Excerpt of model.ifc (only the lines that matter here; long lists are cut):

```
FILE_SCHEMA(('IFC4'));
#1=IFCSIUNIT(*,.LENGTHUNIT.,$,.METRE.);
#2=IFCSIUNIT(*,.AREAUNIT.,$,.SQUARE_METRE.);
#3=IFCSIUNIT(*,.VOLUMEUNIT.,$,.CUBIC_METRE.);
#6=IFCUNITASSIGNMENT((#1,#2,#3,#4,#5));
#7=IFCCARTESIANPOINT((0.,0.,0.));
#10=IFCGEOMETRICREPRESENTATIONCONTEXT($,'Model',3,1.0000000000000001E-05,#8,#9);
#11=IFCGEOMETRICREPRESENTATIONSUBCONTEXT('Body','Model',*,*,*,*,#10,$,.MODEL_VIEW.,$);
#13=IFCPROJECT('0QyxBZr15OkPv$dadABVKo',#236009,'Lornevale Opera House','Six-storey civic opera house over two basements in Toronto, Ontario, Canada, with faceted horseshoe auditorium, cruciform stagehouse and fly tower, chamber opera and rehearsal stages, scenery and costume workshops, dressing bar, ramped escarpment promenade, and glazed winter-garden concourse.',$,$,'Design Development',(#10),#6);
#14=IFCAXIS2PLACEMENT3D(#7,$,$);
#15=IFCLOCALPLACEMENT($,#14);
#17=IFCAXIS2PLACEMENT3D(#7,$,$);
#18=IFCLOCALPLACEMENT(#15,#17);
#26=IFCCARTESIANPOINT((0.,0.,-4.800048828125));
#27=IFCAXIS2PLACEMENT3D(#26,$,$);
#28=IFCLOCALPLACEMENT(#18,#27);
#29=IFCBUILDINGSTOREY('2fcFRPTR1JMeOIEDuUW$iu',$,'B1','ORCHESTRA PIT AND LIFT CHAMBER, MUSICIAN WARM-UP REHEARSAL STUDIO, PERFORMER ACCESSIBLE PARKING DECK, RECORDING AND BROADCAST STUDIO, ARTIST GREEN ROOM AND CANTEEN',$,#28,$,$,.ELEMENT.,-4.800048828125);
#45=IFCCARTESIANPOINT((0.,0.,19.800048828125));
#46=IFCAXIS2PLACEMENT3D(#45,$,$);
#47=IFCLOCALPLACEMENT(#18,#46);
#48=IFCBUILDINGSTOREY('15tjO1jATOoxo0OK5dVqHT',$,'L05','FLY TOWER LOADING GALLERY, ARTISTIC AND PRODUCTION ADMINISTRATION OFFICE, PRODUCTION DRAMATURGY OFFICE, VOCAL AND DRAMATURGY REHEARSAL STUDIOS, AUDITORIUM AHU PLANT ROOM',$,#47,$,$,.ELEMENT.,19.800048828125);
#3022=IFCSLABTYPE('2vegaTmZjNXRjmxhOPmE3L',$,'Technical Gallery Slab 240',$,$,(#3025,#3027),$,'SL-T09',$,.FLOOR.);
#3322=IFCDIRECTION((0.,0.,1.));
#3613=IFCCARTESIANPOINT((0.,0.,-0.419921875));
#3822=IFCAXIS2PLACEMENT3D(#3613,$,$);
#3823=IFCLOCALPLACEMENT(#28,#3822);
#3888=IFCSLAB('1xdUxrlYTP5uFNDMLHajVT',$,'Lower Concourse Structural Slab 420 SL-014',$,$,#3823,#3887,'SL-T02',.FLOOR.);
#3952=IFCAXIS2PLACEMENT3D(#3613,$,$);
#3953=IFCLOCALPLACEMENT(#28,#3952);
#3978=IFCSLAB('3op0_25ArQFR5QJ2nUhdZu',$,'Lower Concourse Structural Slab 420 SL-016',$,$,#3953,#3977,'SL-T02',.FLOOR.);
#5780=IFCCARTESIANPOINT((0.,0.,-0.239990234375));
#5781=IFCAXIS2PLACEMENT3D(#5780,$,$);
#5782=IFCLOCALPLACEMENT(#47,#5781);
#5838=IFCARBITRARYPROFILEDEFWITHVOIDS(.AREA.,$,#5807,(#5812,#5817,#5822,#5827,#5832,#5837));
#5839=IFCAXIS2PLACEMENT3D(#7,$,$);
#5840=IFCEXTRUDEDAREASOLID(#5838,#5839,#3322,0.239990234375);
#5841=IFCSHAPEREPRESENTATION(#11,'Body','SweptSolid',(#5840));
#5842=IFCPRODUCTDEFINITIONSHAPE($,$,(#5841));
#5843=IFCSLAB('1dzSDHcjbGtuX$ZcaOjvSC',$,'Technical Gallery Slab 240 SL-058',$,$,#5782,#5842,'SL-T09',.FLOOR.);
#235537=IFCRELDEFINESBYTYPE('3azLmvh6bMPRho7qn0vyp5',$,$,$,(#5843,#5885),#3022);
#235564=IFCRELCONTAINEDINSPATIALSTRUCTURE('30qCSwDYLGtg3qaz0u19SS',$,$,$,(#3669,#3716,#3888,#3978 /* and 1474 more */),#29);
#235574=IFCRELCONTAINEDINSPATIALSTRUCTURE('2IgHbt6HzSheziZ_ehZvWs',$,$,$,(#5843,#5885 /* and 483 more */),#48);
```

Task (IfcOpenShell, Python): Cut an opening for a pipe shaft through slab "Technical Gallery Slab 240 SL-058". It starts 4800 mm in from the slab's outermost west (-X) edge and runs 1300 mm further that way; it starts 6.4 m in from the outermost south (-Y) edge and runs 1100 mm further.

```python
import numpy as np
import ifcopenshell
import ifcopenshell.api.feature
import ifcopenshell.api.geometry
import ifcopenshell.api.root
import ifcopenshell.geom
import ifcopenshell.util.placement
import ifcopenshell.util.representation
import ifcopenshell.util.shape
import ifcopenshell.util.unit

model = ifcopenshell.open("model.ifc")
unit_scale = ifcopenshell.util.unit.calculate_unit_scale(model)
settings = ifcopenshell.geom.settings()


def volume(element):
    """Net volume in cubic metres, openings subtracted."""
    shape = ifcopenshell.geom.create_shape(settings, element)
    return ifcopenshell.util.shape.get_volume(shape.geometry)


slab = model.by_id(5843)
before = volume(slab)

# Extent in the slab's own axes, in metres. The edges named are its -X and -Y sides.
slab_shape = ifcopenshell.geom.create_shape(settings, slab)
vertices = ifcopenshell.util.shape.get_vertices(slab_shape.geometry)
x_min, y_min, bottom = vertices.min(axis=0)
top = vertices[:, 2].max()

opening = ifcopenshell.api.root.create_entity(model, ifc_class="IfcOpeningElement", name="Pipe shaft opening", predefined_type="OPENING")
context = ifcopenshell.util.representation.get_context(model, "Model", "Body", "MODEL_VIEW")
width, depth = 1.3, 1.1
outline = [(0.0, 0.0), (width, 0.0), (width, depth), (0.0, depth), (0.0, 0.0)]
# Overshoot both faces by 50 mm so the cut is clean.
shape = ifcopenshell.api.geometry.add_slab_representation(
    model, context=context, depth=top - bottom + 0.1, polyline=outline
)
ifcopenshell.api.geometry.assign_representation(model, product=opening, representation=shape)

matrix = ifcopenshell.util.placement.get_local_placement(slab.ObjectPlacement)
matrix[:, 3] = matrix @ np.append(np.array([x_min + 4.8, y_min + 6.4, bottom - 0.05]) / unit_scale, 1.0)
ifcopenshell.api.geometry.edit_object_placement(model, product=opening, matrix=matrix, is_si=False)
ifcopenshell.api.feature.add_feature(model, feature=opening, element=slab)

after = volume(slab)

print(f"slab volume {before:.3f} -> {after:.3f} m3")

model.write("model_updated.ifc")
```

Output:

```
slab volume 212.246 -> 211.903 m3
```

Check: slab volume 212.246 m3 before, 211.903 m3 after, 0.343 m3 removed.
